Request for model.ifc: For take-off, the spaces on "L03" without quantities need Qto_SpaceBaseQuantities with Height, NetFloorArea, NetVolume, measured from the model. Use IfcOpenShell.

First a look at what the model holds.

```python
import ifcopenshell
import ifcopenshell.util.element
import ifcopenshell.util.unit

model = ifcopenshell.open("model.ifc")
print(model.schema)
for unit_type in ("LENGTHUNIT", "AREAUNIT", "VOLUMEUNIT"):
    print(unit_type, ifcopenshell.util.unit.calculate_unit_scale(model, unit_type))
storey = next(s for s in model.by_type("IfcBuildingStorey") if s.Name == "L03")
spaces = [e for e in ifcopenshell.util.element.get_decomposition(storey) if e.is_a("IfcSpace")]
for e in sorted(spaces, key=lambda e: e.id()):
    print(e.id(), e.is_a(), e.Name, list(ifcopenshell.util.element.get_psets(e, qtos_only=True)), sep=" | ")
```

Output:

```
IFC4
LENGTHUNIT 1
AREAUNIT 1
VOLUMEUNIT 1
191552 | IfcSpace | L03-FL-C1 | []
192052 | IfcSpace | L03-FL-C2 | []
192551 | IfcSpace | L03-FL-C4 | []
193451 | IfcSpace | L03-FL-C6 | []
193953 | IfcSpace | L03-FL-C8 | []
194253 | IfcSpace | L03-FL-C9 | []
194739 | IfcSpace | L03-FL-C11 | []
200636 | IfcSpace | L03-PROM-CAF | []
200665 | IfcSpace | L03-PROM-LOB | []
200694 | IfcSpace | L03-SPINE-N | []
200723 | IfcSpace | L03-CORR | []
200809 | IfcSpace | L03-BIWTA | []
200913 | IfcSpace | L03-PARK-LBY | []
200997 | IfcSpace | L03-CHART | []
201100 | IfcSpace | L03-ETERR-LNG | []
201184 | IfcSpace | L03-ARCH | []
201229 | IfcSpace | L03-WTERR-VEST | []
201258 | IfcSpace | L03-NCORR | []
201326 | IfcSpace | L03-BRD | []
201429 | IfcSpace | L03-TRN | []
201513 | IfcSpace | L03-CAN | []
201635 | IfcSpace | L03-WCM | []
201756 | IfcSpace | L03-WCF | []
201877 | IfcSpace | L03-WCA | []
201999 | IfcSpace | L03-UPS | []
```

```python
import ifcopenshell
import ifcopenshell.api.pset
import ifcopenshell.geom
import ifcopenshell.util.element
import ifcopenshell.util.shape
import ifcopenshell.util.unit

model = ifcopenshell.open("model.ifc")
unit_scale = ifcopenshell.util.unit.calculate_unit_scale(model)
area_scale = ifcopenshell.util.unit.calculate_unit_scale(model, "AREAUNIT")
volume_scale = ifcopenshell.util.unit.calculate_unit_scale(model, "VOLUMEUNIT")
settings = ifcopenshell.geom.settings()

storey = next(s for s in model.by_type("IfcBuildingStorey") if s.Name == "L03")
spaces = [e for e in ifcopenshell.util.element.get_decomposition(storey) if e.is_a("IfcSpace")]

for e in sorted(spaces, key=lambda e: e.id()):
    if ifcopenshell.util.element.get_psets(e, qtos_only=True, should_inherit=False):
        continue
    # Geometry comes back in metres, in the element's own axes.
    shape = ifcopenshell.geom.create_shape(settings, e)
    values = {
        "Height": ifcopenshell.util.shape.get_z(shape.geometry) / unit_scale,
        "NetFloorArea": ifcopenshell.util.shape.get_footprint_area(shape.geometry) / area_scale,
        "NetVolume": ifcopenshell.util.shape.get_volume(shape.geometry) / volume_scale,
    }
    qto = ifcopenshell.api.pset.add_qto(model, product=e, name="Qto_SpaceBaseQuantities")
    ifcopenshell.api.pset.edit_qto(model, qto=qto, properties=values)
    print(e.id(), {k: round(v, 3) for k, v in values.items()})

model.write("model_updated.ifc")
```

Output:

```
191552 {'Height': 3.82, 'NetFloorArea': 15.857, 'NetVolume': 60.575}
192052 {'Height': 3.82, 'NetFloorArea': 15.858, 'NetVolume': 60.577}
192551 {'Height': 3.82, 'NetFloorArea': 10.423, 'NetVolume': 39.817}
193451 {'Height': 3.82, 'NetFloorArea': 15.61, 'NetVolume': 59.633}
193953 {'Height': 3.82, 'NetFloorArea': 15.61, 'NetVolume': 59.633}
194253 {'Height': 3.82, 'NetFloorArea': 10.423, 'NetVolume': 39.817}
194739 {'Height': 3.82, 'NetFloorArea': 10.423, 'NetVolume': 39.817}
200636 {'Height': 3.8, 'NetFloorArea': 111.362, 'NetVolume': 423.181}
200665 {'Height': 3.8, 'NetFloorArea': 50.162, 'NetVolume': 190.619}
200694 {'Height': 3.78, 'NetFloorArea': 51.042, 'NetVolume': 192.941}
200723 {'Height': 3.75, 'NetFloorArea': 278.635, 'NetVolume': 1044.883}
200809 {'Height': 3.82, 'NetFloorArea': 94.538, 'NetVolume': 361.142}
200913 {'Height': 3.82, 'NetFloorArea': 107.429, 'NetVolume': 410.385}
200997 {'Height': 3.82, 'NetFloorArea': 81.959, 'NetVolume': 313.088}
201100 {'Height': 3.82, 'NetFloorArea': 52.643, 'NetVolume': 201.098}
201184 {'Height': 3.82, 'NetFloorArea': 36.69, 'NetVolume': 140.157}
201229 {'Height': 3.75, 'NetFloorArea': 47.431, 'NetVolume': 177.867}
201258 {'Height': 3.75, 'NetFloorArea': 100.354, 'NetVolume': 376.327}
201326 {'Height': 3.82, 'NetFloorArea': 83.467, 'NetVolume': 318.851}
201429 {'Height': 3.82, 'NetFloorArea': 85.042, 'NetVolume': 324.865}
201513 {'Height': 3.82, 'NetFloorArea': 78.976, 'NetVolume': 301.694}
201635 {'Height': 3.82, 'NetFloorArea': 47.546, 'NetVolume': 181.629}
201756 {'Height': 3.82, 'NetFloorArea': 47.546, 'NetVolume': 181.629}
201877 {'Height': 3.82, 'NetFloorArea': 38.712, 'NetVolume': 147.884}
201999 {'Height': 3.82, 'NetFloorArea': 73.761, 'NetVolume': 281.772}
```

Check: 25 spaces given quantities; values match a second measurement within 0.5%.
